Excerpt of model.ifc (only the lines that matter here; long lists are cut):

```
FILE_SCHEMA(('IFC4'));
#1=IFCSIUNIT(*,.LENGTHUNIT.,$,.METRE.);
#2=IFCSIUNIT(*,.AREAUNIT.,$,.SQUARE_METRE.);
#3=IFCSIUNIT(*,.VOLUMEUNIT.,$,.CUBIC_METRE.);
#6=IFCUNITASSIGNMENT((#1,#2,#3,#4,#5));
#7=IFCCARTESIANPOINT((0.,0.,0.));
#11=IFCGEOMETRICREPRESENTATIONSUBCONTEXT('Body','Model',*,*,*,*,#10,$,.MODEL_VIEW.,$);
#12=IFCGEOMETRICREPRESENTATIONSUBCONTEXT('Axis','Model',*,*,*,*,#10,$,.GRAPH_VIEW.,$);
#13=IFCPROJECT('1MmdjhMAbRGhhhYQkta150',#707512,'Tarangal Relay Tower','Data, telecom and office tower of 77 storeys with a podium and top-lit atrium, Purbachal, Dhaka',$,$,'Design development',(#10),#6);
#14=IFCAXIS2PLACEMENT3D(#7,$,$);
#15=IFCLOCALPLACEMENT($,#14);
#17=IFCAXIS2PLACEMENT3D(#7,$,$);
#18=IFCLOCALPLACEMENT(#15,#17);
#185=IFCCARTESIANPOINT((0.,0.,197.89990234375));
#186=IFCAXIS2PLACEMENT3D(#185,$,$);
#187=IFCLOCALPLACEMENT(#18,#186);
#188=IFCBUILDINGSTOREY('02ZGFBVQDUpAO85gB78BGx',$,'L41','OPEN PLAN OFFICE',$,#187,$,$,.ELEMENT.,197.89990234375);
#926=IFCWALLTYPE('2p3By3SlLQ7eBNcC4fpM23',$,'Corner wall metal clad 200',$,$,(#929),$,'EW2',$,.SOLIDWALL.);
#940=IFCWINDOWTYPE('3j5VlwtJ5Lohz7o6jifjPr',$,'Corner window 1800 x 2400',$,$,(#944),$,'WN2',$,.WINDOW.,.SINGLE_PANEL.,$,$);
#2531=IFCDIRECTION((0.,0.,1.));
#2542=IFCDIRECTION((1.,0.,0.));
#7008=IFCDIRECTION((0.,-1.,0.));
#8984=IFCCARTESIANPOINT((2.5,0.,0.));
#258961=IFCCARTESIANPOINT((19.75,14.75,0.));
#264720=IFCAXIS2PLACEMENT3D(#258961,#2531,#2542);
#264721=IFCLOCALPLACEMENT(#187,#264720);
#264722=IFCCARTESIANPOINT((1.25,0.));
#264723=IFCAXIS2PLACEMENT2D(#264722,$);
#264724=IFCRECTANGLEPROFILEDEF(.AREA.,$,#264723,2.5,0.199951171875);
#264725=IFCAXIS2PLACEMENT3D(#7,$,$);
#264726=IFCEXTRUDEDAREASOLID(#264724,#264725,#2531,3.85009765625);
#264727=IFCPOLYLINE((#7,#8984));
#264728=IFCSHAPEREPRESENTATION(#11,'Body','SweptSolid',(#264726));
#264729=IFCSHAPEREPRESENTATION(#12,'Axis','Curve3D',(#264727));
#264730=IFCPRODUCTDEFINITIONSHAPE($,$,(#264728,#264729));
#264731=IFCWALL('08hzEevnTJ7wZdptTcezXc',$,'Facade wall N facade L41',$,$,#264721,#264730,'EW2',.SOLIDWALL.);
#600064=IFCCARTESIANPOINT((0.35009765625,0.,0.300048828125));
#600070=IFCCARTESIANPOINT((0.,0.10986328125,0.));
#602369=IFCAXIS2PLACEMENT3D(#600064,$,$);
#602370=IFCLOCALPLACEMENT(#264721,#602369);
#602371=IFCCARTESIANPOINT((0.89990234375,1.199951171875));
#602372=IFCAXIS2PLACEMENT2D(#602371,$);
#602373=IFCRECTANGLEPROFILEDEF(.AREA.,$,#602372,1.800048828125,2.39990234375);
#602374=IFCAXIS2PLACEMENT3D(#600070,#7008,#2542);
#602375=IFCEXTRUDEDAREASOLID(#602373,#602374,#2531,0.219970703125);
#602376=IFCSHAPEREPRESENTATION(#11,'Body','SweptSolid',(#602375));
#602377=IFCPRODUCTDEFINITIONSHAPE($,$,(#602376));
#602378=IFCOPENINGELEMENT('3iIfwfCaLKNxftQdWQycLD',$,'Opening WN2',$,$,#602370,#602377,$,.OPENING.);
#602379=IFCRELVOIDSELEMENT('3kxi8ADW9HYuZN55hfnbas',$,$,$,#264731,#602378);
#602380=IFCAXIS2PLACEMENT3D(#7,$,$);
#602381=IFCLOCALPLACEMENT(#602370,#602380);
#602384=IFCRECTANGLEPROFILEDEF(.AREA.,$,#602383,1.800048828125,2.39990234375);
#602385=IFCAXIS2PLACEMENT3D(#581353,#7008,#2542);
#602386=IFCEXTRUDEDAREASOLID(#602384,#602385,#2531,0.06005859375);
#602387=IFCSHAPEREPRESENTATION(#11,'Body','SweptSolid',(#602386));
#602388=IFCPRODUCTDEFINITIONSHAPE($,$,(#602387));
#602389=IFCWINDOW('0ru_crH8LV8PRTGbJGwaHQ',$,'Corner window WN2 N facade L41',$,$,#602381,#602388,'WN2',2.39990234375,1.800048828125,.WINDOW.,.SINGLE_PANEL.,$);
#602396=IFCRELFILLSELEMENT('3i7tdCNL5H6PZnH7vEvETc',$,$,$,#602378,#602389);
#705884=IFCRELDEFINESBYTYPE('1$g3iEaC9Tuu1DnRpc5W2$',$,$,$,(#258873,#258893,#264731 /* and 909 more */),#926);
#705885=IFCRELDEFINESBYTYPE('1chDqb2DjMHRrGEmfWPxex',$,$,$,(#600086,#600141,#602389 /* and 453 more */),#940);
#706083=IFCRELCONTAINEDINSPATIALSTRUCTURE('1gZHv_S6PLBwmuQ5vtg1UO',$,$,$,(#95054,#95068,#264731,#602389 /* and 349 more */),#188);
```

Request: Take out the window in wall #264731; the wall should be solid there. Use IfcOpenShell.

```python
import ifcopenshell
import ifcopenshell.api.feature
import ifcopenshell.api.root
import ifcopenshell.geom
import ifcopenshell.util.shape

model = ifcopenshell.open("model.ifc")
settings = ifcopenshell.geom.settings()


def volume(element):
    """Net volume in cubic metres, openings subtracted."""
    shape = ifcopenshell.geom.create_shape(settings, element)
    return ifcopenshell.util.shape.get_volume(shape.geometry)


window = model.by_guid("0ru_crH8LV8PRTGbJGwaHQ")
opening = window.FillsVoids[0].RelatingOpeningElement
wall = opening.VoidsElements[0].RelatingBuildingElement
before = volume(wall)

ifcopenshell.api.root.remove_product(model, product=window)
ifcopenshell.api.feature.remove_feature(model, feature=opening)

after = volume(wall)

print(f"wall volume {before:.3f} -> {after:.3f} m3")

model.write("model_rev.ifc")
```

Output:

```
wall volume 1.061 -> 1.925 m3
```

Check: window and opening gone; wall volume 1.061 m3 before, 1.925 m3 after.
